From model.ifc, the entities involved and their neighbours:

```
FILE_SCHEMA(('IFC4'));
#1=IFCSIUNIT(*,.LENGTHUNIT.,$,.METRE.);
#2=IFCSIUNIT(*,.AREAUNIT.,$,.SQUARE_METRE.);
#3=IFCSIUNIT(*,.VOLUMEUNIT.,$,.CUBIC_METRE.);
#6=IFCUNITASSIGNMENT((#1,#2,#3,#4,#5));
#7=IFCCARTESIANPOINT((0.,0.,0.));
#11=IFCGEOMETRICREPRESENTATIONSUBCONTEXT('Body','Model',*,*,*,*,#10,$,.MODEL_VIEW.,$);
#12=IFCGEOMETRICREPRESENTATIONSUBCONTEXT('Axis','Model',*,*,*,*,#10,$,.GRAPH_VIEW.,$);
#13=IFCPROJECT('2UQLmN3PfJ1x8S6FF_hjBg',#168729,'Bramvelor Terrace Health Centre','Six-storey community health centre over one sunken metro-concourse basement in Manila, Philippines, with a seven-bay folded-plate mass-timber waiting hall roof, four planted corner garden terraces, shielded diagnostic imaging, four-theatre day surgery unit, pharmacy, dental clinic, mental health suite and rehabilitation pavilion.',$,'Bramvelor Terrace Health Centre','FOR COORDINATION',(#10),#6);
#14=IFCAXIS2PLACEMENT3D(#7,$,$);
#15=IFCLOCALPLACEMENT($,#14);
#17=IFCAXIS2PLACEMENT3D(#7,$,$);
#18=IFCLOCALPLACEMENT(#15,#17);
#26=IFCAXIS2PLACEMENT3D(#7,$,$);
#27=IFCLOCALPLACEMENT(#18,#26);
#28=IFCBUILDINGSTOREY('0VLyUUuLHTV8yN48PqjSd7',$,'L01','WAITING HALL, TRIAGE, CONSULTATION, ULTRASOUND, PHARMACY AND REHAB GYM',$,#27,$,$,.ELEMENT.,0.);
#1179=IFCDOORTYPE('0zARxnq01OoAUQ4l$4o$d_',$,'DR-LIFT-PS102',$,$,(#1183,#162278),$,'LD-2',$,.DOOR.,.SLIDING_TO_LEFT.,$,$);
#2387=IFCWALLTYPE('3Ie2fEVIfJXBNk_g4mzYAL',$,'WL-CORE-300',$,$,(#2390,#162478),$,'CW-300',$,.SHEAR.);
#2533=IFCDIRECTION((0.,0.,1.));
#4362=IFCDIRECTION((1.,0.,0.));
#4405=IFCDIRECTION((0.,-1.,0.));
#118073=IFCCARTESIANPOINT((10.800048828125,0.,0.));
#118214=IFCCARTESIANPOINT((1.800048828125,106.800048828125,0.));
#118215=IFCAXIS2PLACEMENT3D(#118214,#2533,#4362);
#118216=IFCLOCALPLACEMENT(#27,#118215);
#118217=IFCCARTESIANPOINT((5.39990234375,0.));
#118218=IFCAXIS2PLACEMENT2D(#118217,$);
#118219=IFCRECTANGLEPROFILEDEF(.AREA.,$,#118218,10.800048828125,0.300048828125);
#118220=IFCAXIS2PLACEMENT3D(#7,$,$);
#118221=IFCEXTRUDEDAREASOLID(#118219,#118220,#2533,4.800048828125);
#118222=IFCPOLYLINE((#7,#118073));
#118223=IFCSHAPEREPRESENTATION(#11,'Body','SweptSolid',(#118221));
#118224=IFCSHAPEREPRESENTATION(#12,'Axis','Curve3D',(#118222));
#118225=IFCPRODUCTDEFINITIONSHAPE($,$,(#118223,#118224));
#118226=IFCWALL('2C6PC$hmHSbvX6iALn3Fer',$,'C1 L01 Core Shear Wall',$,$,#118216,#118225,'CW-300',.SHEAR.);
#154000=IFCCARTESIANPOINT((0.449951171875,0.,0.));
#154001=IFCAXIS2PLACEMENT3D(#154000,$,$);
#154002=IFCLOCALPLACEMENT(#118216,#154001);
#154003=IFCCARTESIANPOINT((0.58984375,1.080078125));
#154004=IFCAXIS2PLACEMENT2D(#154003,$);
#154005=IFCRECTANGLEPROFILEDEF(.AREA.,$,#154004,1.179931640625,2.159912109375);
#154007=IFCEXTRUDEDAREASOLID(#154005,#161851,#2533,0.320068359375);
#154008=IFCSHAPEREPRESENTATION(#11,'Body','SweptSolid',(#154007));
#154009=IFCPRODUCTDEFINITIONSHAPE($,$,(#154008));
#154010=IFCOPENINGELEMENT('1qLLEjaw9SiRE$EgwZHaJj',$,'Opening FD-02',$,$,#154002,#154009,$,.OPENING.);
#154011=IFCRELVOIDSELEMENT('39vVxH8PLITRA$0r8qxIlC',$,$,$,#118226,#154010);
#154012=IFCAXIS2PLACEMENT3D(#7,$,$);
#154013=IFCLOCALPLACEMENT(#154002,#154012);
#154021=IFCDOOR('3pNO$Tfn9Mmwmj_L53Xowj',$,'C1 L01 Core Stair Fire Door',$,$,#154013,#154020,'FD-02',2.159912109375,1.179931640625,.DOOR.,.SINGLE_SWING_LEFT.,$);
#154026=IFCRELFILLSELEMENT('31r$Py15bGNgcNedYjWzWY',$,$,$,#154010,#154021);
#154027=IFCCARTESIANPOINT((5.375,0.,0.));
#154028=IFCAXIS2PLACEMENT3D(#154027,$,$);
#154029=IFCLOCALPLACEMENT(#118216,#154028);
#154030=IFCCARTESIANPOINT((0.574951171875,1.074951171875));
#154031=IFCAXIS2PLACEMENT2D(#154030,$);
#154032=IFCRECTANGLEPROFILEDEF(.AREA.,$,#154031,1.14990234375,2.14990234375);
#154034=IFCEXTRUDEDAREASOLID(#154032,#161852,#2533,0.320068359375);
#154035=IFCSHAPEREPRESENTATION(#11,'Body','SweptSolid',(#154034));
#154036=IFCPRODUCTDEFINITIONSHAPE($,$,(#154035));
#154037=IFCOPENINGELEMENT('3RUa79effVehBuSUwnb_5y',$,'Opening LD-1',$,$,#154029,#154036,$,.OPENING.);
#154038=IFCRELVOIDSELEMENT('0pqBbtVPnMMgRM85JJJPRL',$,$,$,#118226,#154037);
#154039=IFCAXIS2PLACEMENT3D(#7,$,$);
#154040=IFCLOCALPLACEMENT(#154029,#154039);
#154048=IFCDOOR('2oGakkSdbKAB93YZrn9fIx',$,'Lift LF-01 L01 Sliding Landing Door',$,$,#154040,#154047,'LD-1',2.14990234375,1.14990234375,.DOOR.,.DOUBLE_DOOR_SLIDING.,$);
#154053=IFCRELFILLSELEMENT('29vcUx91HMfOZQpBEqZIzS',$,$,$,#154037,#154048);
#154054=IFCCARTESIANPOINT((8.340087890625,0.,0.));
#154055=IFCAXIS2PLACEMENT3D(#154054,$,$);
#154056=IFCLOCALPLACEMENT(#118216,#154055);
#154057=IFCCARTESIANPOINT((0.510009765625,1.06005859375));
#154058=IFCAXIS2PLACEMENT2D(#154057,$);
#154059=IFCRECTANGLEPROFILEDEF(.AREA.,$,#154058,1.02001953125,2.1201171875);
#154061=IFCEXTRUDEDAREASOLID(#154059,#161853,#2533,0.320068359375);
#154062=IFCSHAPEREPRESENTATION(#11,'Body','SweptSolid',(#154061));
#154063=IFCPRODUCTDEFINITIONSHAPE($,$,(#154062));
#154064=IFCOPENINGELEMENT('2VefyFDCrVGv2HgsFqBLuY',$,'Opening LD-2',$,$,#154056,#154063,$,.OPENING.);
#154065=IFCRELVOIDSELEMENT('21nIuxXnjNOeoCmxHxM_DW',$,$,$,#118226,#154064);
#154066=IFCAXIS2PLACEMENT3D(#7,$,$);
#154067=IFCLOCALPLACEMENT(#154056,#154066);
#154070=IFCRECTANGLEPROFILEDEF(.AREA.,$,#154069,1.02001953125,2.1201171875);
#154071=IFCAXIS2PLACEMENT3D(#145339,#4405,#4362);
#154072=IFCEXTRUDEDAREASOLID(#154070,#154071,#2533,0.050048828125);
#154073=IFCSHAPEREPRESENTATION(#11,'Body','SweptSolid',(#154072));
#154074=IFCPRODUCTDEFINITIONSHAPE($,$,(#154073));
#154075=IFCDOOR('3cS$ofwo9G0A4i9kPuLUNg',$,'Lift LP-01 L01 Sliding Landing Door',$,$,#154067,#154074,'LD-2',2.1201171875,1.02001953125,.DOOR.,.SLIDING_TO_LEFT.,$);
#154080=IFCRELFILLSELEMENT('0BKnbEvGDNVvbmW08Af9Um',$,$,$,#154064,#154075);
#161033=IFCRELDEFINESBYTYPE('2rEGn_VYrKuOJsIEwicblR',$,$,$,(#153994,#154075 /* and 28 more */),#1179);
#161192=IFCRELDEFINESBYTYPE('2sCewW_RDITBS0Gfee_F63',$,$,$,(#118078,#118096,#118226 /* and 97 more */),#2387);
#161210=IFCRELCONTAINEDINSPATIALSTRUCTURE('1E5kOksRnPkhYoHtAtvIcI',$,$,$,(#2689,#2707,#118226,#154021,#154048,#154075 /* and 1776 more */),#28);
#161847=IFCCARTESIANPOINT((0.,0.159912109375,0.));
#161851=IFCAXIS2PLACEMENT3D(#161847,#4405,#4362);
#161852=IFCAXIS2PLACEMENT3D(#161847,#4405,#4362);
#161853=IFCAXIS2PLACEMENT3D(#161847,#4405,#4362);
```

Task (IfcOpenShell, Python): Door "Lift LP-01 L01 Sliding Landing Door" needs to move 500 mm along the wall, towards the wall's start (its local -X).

```python
import ifcopenshell
import ifcopenshell.api.geometry
import ifcopenshell.util.placement
import ifcopenshell.util.unit

model = ifcopenshell.open("model.ifc")
unit_scale = ifcopenshell.util.unit.calculate_unit_scale(model)

door = model.by_id(154075)
opening = door.FillsVoids[0].RelatingOpeningElement
wall = opening.VoidsElements[0].RelatingBuildingElement

wall_matrix = ifcopenshell.util.placement.get_local_placement(wall.ObjectPlacement)
shift = wall_matrix[:3, 0] * -0.5 / unit_scale
before = ifcopenshell.util.placement.get_local_placement(door.ObjectPlacement)[:3, 3].copy()

# The door is placed relative to its opening, so it follows when the opening moves.
matrix = ifcopenshell.util.placement.get_local_placement(opening.ObjectPlacement)
matrix[:3, 3] += shift
ifcopenshell.api.geometry.edit_object_placement(
    model, product=opening, matrix=matrix, is_si=False, should_transform_children=True
)

after = ifcopenshell.util.placement.get_local_placement(door.ObjectPlacement)[:3, 3]
print("door moved by", (after - before).round(3) + 0.0)

model.write("model_v2.ifc")
```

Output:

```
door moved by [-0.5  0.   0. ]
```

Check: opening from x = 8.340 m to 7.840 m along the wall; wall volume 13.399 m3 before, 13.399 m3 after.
